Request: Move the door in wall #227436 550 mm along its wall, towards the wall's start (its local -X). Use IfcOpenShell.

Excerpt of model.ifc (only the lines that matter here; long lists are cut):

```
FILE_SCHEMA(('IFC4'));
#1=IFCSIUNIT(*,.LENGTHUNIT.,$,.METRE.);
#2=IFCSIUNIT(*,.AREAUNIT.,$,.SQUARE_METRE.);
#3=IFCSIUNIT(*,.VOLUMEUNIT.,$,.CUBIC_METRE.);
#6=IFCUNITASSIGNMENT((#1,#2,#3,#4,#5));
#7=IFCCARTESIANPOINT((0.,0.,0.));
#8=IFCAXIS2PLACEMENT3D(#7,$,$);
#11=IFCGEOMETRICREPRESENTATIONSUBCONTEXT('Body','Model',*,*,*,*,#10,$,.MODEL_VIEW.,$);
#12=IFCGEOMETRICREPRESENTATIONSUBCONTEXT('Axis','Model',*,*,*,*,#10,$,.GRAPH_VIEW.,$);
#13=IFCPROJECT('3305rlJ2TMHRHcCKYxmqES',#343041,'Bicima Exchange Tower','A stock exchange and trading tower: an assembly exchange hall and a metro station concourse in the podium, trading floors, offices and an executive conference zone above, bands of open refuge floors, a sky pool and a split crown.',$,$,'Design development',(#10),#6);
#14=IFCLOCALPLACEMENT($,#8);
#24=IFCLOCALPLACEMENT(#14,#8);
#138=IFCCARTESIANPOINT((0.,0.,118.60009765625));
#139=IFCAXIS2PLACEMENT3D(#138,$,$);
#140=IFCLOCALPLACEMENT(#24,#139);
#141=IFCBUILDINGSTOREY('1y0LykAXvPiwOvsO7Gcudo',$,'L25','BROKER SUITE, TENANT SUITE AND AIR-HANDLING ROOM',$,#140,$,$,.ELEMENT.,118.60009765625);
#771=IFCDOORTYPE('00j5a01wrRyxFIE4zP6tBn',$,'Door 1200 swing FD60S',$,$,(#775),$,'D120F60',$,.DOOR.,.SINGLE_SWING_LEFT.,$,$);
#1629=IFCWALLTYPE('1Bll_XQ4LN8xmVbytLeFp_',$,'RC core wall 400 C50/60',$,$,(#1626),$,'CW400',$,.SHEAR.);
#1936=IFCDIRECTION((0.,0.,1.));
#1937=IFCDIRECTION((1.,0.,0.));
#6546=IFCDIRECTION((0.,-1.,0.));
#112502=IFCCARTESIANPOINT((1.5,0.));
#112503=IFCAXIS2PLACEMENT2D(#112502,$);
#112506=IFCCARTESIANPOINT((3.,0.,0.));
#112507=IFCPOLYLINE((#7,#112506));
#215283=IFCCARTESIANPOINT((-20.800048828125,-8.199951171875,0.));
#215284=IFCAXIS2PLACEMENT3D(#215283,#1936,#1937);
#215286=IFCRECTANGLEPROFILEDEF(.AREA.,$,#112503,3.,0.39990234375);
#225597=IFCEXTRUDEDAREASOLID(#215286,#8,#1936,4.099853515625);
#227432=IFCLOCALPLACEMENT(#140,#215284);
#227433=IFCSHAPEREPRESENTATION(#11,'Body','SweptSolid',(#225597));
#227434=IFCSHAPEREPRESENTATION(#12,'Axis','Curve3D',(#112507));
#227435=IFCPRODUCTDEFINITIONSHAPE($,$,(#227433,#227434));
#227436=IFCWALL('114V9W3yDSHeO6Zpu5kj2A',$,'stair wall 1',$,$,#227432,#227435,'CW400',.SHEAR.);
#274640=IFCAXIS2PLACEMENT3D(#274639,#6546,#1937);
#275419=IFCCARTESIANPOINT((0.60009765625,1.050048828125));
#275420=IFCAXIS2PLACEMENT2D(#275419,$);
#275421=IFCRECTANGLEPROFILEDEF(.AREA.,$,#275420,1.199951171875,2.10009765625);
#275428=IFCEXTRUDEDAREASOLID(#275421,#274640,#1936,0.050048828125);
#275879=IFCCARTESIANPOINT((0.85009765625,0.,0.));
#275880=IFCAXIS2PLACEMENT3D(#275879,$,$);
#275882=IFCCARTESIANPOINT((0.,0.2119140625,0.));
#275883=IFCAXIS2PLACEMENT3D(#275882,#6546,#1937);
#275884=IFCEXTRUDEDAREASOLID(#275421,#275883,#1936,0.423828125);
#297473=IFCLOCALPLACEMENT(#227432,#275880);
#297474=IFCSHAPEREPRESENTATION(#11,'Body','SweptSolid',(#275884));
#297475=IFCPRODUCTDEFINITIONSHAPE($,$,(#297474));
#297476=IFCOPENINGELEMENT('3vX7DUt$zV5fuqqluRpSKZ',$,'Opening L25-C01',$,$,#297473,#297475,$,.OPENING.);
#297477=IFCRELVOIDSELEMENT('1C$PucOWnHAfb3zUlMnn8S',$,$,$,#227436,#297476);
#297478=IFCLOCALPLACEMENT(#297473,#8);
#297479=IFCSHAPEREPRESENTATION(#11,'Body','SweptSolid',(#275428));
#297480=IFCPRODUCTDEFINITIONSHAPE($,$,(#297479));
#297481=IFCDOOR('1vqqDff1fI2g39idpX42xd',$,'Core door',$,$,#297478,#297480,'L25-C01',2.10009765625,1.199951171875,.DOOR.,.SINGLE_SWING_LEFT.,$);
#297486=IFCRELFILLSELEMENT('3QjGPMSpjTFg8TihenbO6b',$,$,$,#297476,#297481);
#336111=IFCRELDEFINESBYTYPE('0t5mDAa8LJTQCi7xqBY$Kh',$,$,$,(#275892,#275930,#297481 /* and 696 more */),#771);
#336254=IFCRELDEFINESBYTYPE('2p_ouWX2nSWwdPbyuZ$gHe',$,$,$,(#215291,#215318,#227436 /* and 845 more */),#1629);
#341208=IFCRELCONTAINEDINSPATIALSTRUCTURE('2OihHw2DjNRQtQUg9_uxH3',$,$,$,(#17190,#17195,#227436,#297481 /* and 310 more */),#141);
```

```python
import ifcopenshell
import ifcopenshell.api.geometry
import ifcopenshell.util.placement

model = ifcopenshell.open("model.ifc")

door = model.by_guid("1vqqDff1fI2g39idpX42xd")
opening = door.FillsVoids[0].RelatingOpeningElement
wall = opening.VoidsElements[0].RelatingBuildingElement

wall_matrix = ifcopenshell.util.placement.get_local_placement(wall.ObjectPlacement)
shift = wall_matrix[:3, 0] * -0.55
before = ifcopenshell.util.placement.get_local_placement(door.ObjectPlacement)[:3, 3].copy()

# The door is placed relative to its opening, so it follows when the opening moves.
matrix = ifcopenshell.util.placement.get_local_placement(opening.ObjectPlacement)
matrix[:3, 3] += shift
ifcopenshell.api.geometry.edit_object_placement(
    model, product=opening, matrix=matrix, is_si=False, should_transform_children=True
)

after = ifcopenshell.util.placement.get_local_placement(door.ObjectPlacement)[:3, 3]
print("door moved by", (after - before).round(3) + 0.0)

model.write("model_rev.ifc")
```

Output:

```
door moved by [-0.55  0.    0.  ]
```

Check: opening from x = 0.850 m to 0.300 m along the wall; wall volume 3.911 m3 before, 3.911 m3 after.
